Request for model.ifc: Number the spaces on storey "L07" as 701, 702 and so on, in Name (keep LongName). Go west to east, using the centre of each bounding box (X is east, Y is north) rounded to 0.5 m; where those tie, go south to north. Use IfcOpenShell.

First a look at what the model holds.

```python
import ifcopenshell
import ifcopenshell.util.element
import ifcopenshell.util.placement

model = ifcopenshell.open("model.ifc")
print(model.schema)
storey = next(s for s in model.by_type("IfcBuildingStorey") if s.Name == "L07")
spaces = [e for e in ifcopenshell.util.element.get_decomposition(storey) if e.is_a("IfcSpace")]
for e in sorted(spaces, key=lambda e: e.id()):
    origin = ifcopenshell.util.placement.get_local_placement(e.ObjectPlacement)[:3, 3]
    print(e.id(), e.Name, e.LongName, origin.round(2) + 0.0, sep=" | ")
```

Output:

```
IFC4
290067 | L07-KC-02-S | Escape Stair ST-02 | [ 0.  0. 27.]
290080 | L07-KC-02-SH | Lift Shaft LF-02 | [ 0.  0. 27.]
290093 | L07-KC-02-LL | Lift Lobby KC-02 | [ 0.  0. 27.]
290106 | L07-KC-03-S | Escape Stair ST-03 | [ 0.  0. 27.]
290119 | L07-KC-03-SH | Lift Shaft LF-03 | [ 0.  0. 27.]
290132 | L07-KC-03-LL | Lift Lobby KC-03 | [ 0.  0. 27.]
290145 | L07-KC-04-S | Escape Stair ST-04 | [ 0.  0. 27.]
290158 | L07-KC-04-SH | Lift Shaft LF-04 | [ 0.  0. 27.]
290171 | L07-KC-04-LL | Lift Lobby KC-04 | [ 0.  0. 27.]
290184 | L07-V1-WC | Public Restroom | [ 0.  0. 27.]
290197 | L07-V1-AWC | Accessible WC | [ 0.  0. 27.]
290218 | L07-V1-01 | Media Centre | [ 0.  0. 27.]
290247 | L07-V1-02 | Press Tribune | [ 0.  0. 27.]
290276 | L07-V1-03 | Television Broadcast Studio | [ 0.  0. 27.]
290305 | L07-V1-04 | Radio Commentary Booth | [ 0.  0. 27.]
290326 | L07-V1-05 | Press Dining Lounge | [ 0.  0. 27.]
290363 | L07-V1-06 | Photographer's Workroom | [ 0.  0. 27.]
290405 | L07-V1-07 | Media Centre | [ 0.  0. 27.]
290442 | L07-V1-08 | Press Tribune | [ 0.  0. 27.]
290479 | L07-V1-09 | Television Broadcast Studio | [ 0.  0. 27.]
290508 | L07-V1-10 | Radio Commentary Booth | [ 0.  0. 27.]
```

```python
import ifcopenshell
import ifcopenshell.geom
import ifcopenshell.util.element
import ifcopenshell.util.shape

model = ifcopenshell.open("model.ifc")
settings = ifcopenshell.geom.settings()
settings.set("use-world-coords", True)


def centre(element):
    shape = ifcopenshell.geom.create_shape(settings, element)
    return ifcopenshell.util.shape.get_bbox_centroid(shape.geometry)


storey = next(s for s in model.by_type("IfcBuildingStorey") if s.Name == "L07")
spaces = [e for e in ifcopenshell.util.element.get_decomposition(storey) if e.is_a("IfcSpace")]

# Insertion points can sit at a corner or the storey origin, so sort by the geometry (in metres).
centres = {e: centre(e) for e in spaces}
spaces.sort(key=lambda e: (round(centres[e][0] / 0.5), centres[e][1]))

for i, e in enumerate(spaces, start=1):
    number = f"7{i:02d}"
    e.Name = number
    print(e.id(), number)

model.write("model-out.ifc")
```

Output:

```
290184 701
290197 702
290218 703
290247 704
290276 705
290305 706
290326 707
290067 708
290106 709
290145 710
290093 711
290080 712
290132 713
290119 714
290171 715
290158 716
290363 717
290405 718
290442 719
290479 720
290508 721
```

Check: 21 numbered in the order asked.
